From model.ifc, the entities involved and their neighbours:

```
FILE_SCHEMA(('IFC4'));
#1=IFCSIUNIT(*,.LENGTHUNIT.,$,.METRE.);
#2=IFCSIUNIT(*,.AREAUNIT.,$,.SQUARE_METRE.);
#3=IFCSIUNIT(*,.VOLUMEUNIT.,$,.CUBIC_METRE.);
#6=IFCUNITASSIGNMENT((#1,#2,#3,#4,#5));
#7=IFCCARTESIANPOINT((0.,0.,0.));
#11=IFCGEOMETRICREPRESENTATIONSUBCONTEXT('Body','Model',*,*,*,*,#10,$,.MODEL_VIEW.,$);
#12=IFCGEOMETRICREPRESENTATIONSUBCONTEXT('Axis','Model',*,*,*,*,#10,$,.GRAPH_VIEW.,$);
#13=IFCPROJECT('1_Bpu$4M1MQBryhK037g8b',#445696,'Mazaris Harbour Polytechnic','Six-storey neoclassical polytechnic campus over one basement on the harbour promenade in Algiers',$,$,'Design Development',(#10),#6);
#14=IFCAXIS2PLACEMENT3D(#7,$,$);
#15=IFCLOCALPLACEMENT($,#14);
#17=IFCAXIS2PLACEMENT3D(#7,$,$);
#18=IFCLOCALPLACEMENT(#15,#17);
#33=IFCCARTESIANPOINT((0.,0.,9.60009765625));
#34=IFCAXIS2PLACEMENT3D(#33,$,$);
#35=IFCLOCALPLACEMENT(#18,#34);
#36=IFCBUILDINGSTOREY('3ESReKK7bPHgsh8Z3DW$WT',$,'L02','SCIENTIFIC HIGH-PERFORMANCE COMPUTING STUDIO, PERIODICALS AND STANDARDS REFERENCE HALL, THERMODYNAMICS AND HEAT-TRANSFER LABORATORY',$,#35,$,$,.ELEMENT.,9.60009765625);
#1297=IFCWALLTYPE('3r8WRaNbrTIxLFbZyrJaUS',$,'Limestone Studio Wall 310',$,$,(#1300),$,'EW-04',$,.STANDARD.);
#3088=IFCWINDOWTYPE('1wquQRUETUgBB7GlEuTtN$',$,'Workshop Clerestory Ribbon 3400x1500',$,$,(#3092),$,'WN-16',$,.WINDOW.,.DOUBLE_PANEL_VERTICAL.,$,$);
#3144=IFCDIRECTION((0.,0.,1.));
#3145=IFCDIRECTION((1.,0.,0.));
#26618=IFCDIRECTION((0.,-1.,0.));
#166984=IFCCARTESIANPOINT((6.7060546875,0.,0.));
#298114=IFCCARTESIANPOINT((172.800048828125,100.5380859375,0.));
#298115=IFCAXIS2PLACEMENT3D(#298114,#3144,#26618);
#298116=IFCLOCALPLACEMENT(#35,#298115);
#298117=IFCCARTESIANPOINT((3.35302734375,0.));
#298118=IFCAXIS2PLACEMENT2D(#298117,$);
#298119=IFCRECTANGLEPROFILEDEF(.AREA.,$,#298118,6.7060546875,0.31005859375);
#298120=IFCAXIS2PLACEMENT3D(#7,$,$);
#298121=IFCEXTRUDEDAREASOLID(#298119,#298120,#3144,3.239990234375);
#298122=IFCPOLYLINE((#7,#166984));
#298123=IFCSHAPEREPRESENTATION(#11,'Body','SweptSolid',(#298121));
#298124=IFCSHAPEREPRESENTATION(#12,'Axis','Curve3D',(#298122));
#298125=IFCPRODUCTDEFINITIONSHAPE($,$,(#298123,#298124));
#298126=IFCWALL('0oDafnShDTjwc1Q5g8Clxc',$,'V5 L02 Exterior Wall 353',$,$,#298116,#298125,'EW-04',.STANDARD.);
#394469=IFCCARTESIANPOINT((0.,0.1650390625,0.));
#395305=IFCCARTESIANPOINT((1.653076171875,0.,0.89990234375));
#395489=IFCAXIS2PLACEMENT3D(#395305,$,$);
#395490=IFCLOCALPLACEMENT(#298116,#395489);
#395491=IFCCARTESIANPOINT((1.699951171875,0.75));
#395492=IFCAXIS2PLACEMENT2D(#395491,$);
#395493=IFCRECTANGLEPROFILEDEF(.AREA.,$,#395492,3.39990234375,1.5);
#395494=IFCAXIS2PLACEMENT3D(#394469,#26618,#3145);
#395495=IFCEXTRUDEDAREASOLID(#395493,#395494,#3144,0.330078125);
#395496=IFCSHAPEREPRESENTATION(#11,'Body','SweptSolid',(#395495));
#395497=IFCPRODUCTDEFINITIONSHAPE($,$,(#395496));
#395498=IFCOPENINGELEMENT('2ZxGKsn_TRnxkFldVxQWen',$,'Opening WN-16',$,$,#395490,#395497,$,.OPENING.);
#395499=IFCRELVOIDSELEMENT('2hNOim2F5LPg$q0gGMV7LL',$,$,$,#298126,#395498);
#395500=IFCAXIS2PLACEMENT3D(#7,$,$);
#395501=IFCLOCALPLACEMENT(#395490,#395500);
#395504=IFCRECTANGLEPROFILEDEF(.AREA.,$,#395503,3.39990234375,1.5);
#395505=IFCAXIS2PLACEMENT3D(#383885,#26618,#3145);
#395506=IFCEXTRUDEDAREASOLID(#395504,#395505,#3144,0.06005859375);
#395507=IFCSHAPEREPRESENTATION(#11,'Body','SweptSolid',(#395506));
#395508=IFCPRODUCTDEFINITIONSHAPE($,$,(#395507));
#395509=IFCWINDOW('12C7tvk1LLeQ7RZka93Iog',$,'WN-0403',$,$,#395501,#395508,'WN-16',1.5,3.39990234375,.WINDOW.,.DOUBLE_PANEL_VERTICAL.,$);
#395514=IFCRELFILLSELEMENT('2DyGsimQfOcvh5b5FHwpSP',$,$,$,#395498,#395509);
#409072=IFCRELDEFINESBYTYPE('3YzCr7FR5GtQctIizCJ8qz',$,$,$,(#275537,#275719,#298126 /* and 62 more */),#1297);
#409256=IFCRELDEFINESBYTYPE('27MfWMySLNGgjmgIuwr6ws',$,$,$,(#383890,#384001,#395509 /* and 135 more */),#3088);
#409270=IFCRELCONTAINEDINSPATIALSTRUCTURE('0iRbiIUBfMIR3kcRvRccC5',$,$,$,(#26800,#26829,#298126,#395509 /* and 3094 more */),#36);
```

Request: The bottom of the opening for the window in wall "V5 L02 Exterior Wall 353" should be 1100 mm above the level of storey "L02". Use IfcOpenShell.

```python
import numpy as np
import ifcopenshell
import ifcopenshell.api.geometry
import ifcopenshell.geom
import ifcopenshell.util.element
import ifcopenshell.util.placement
import ifcopenshell.util.shape
import ifcopenshell.util.unit

model = ifcopenshell.open("model.ifc")
unit_scale = ifcopenshell.util.unit.calculate_unit_scale(model)

window = model.by_id(395509)
opening = window.FillsVoids[0].RelatingOpeningElement
storey = ifcopenshell.util.element.get_container(window, ifc_class="IfcBuildingStorey")
level = ifcopenshell.util.placement.get_local_placement(storey.ObjectPlacement)[2, 3]

# The opening's origin need not be at the sill, so measure its lowest point.
shape = ifcopenshell.geom.create_shape(ifcopenshell.geom.settings(), opening)
bottom = ifcopenshell.util.shape.get_shape_bottom_elevation(shape, shape.geometry) / unit_scale
dz = level + 1.1 - bottom

shift = np.array([0.0, 0.0, dz])
# The window is placed relative to its opening, so it follows when the opening moves.
matrix = ifcopenshell.util.placement.get_local_placement(opening.ObjectPlacement)
matrix[:3, 3] += shift
ifcopenshell.api.geometry.edit_object_placement(
    model, product=opening, matrix=matrix, is_si=False, should_transform_children=True
)

print(f"moved by {dz * unit_scale:+.3f} m")

model.write("model_updated.ifc")
```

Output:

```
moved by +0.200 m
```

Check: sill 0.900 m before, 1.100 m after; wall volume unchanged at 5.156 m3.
